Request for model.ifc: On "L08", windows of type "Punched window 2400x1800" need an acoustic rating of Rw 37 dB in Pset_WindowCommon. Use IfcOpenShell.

First a look at what the model holds.

```python
import ifcopenshell
import ifcopenshell.util.element

model = ifcopenshell.open("model.ifc")
print(model.schema)
storey = next(s for s in model.by_type("IfcBuildingStorey") if s.Name == "L08")
windows = [e for e in ifcopenshell.util.element.get_decomposition(storey) if e.is_a("IfcWindow")]
seen = {}
for e in windows:
    element_type = ifcopenshell.util.element.get_type(e)
    key = (element_type.Name if element_type != e and element_type else None, ifcopenshell.util.element.get_pset(e, "Pset_WindowCommon", "AcousticRating"))
    seen[key] = seen.get(key, 0) + 1
for (name, value), count in sorted(seen.items(), key=str):
    print(count, "x", name, "|", value)
```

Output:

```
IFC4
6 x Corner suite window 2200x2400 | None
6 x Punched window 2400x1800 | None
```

```python
import ifcopenshell
import ifcopenshell.api.pset
import ifcopenshell.util.element

model = ifcopenshell.open("model.ifc")

storey = next(s for s in model.by_type("IfcBuildingStorey") if s.Name == "L08")
windows = [e for e in ifcopenshell.util.element.get_decomposition(storey) if e.is_a("IfcWindow")]

count = 0
for e in windows:
    element_type = ifcopenshell.util.element.get_type(e)
    if element_type in (None, e) or element_type.Name != "Punched window 2400x1800":
        continue
    found = ifcopenshell.util.element.get_pset(e, "Pset_WindowCommon", should_inherit=False)
    if found:
        pset = model.by_id(found["id"])
        if len(ifcopenshell.util.element.get_elements_by_pset(pset)) > 1:
            pset = ifcopenshell.api.pset.unshare_pset(model, products=[e], pset=pset)[0]
    else:
        pset = ifcopenshell.api.pset.add_pset(model, product=e, name="Pset_WindowCommon")
    ifcopenshell.api.pset.edit_pset(model, pset=pset, properties={"AcousticRating": "Rw 37 dB"})
    count += 1

print(count, "windows updated")

model.write("model_edited.ifc")
```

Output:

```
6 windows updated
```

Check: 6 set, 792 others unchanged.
